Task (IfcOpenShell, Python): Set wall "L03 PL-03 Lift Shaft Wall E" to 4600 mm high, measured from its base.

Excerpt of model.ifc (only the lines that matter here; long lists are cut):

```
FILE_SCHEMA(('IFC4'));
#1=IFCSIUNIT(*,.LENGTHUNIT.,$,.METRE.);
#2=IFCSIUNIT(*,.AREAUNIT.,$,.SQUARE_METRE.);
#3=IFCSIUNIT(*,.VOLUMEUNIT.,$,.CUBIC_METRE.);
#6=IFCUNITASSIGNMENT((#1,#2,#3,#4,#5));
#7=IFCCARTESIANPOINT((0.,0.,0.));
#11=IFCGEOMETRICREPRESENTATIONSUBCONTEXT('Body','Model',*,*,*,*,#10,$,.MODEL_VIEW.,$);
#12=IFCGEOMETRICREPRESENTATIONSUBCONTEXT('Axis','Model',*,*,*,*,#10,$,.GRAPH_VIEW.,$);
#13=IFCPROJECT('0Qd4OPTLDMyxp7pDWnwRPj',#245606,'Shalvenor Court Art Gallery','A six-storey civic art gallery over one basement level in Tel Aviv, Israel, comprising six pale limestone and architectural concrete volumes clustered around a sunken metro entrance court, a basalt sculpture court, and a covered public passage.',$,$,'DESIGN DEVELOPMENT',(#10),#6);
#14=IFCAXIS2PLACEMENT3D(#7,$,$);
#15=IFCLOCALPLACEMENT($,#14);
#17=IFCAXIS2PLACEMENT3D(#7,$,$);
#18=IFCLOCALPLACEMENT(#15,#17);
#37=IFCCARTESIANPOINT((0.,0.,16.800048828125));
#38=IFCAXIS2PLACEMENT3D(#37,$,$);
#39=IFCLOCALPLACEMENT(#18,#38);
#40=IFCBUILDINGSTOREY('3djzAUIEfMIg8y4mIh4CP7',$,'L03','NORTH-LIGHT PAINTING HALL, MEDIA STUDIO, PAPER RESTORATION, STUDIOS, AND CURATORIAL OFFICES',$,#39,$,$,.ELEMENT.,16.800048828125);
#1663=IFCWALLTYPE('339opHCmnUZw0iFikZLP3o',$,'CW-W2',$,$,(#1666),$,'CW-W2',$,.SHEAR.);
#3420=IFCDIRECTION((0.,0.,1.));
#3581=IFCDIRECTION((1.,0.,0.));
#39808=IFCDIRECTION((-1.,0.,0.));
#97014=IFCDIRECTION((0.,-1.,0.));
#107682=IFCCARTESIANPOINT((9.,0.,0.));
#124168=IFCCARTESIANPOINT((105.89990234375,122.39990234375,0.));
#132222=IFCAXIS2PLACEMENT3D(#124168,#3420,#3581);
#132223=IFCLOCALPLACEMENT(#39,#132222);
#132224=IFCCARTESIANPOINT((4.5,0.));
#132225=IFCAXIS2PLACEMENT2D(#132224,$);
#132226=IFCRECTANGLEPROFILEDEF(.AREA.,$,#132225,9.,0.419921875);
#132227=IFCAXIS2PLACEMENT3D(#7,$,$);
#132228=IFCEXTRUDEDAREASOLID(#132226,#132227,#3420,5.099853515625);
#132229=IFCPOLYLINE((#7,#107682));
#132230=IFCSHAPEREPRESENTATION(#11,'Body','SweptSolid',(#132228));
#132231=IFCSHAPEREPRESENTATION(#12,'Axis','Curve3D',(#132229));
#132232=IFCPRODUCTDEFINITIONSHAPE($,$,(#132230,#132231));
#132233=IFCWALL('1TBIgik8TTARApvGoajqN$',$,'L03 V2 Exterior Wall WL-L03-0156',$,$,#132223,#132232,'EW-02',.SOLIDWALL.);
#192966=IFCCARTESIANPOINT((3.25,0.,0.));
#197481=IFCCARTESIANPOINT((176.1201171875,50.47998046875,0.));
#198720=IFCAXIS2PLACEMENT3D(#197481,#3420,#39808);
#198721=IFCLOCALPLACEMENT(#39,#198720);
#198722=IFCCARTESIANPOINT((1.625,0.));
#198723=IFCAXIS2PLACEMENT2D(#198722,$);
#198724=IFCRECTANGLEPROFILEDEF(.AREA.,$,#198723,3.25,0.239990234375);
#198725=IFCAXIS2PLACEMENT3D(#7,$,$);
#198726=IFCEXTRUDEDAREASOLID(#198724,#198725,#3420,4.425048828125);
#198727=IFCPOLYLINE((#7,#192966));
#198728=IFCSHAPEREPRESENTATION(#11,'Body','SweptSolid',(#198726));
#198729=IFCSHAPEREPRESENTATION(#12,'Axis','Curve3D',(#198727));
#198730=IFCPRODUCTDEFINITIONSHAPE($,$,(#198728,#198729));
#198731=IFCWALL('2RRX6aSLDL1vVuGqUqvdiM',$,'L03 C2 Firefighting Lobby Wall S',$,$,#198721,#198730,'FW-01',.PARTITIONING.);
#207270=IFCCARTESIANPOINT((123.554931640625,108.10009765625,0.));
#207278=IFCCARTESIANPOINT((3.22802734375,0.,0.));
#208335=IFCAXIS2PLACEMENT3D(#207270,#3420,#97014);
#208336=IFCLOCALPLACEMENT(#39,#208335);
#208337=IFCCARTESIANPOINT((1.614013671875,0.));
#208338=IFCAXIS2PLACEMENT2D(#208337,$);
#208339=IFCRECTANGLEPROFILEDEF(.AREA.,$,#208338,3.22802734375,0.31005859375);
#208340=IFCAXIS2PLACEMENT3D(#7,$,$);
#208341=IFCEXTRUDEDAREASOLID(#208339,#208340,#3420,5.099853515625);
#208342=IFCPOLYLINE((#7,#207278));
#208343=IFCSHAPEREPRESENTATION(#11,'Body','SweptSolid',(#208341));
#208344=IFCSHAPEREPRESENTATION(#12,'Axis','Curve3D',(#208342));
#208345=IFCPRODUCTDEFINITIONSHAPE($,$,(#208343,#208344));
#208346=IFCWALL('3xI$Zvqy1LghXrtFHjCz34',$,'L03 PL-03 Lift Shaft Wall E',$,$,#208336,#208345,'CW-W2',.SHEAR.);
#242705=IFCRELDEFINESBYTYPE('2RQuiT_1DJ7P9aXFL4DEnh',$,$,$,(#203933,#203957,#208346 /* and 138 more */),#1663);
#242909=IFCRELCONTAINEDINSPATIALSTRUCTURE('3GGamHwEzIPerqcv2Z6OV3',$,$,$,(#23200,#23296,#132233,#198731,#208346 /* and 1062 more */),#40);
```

```python
import ifcopenshell
import ifcopenshell.geom
import ifcopenshell.util.representation
import ifcopenshell.util.shape

model = ifcopenshell.open("model.ifc")
settings = ifcopenshell.geom.settings()


def volume(element):
    """Net volume in cubic metres, openings subtracted."""
    shape = ifcopenshell.geom.create_shape(settings, element)
    return ifcopenshell.util.shape.get_volume(shape.geometry)


wall = model.by_id(208346)
before = volume(wall)

body = ifcopenshell.util.representation.get_representation(wall, "Model", "Body")
solid = body.Items[0]
old_height = solid.Depth
solid.Depth = 4.6
after = volume(wall)

print(f"height {old_height:g} -> {solid.Depth:g}, volume {before:.3f} -> {after:.3f} m3")

model.write("model_updated.ifc")
```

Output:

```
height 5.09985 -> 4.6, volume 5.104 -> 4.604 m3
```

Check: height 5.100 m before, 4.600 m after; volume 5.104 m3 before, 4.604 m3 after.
